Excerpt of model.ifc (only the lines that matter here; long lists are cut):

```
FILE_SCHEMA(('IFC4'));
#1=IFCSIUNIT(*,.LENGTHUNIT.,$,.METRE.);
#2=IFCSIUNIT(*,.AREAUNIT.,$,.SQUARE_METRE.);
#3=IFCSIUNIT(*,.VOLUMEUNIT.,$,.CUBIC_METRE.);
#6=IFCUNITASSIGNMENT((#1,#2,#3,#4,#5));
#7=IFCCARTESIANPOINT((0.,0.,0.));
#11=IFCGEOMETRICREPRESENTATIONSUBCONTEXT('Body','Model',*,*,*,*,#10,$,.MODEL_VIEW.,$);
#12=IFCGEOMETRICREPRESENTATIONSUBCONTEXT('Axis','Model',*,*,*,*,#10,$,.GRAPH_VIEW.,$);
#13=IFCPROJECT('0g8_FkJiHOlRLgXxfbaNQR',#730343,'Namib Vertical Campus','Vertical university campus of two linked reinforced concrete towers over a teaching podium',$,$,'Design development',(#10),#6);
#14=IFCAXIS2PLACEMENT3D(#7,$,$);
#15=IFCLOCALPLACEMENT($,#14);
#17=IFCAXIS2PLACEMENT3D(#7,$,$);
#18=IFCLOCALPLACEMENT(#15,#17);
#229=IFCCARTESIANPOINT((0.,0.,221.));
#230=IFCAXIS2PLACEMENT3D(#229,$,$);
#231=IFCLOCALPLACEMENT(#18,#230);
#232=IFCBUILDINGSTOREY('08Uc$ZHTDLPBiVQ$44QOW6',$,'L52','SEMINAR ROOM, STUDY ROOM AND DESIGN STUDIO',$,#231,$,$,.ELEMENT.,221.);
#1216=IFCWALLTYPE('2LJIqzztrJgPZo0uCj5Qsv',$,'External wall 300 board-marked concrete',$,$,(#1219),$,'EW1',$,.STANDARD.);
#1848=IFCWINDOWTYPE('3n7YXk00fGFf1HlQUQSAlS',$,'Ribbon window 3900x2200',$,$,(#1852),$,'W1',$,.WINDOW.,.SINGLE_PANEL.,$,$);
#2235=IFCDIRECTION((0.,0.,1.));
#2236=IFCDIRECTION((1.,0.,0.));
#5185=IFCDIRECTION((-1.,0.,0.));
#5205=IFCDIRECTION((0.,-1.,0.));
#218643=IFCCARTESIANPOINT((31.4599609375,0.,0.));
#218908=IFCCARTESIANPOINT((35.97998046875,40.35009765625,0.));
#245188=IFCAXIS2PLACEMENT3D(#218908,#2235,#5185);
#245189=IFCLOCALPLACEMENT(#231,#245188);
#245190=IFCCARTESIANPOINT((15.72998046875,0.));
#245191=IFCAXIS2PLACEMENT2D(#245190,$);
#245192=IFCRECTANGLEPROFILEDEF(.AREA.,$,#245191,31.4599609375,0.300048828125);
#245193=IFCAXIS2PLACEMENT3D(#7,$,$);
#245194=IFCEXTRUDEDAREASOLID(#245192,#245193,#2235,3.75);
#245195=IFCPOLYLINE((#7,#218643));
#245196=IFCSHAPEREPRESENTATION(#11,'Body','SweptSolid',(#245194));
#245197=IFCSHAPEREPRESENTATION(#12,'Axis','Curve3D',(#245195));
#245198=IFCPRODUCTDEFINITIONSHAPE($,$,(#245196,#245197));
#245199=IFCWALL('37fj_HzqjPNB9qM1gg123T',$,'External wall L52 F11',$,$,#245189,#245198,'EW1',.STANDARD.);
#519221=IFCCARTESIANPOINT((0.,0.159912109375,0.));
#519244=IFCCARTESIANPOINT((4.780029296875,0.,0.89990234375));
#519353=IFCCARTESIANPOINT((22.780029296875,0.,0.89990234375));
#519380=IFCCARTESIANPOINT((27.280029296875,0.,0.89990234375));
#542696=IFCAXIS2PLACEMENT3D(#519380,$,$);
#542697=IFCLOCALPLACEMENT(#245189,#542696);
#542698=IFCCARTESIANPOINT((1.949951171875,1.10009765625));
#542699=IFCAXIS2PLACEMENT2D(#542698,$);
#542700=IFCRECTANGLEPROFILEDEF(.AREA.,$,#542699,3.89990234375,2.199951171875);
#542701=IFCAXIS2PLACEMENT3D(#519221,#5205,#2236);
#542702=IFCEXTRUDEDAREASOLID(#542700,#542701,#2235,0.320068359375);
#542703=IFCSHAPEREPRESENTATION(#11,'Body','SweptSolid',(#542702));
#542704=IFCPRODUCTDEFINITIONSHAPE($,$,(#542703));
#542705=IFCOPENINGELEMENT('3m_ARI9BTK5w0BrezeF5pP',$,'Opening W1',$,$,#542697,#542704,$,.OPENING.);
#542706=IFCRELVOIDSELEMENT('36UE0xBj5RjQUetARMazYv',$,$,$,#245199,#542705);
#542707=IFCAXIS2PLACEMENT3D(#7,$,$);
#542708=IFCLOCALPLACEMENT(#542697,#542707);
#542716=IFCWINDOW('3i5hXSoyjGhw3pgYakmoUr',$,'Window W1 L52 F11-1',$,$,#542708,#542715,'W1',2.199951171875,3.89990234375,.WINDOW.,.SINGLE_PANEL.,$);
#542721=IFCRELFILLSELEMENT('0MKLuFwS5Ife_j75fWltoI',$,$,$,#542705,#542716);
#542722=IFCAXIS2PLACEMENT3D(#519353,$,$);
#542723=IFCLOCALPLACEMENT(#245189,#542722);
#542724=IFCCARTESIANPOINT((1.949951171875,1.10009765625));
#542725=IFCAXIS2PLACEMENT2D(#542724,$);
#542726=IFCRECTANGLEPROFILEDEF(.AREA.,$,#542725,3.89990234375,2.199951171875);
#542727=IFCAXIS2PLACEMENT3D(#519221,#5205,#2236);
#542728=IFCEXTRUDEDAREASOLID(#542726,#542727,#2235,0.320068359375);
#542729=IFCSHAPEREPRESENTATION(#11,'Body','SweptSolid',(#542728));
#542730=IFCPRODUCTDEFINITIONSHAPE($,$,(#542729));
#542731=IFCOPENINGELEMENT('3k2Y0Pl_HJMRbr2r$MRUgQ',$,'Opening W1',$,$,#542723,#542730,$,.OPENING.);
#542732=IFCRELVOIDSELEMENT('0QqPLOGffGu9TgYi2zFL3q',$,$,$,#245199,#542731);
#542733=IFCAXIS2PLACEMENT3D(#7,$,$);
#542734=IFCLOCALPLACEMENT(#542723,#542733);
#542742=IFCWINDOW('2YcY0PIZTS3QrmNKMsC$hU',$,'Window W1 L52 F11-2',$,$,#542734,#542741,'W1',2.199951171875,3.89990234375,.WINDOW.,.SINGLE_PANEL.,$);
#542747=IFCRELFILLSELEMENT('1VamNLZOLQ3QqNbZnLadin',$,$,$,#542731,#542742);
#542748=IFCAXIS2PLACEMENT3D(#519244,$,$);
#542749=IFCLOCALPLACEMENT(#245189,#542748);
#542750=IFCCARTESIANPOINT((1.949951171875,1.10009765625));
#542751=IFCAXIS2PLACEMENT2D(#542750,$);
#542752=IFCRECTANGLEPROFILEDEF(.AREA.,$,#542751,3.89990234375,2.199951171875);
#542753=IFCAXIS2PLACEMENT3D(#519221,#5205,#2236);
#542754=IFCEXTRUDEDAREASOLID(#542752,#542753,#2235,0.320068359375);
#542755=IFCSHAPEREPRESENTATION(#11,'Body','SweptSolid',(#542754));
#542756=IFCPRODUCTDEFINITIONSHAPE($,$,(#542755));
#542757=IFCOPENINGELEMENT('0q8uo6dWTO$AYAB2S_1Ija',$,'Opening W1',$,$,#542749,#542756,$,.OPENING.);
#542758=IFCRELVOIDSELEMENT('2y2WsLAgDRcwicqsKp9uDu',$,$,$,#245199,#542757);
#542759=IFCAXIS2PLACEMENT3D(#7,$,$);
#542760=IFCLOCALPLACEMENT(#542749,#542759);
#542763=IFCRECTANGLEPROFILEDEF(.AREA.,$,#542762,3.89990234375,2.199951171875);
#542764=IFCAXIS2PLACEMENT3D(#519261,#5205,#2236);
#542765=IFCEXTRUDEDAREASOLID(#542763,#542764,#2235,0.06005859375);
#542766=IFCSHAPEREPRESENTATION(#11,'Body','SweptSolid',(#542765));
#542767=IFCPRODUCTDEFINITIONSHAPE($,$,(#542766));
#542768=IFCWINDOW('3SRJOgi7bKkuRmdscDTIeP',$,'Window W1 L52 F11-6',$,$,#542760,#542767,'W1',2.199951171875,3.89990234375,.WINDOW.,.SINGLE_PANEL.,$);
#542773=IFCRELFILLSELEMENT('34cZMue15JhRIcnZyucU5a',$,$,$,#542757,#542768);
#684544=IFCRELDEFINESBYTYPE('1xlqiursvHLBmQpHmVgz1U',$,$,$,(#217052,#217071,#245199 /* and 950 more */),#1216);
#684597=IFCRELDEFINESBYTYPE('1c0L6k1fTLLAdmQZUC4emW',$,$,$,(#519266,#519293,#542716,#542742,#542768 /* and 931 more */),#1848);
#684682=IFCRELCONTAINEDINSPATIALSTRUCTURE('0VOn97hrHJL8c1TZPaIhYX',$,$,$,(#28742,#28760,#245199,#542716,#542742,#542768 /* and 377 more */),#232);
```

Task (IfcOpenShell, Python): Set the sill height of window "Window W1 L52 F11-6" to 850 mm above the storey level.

```python
import numpy as np
import ifcopenshell
import ifcopenshell.api.geometry
import ifcopenshell.geom
import ifcopenshell.util.element
import ifcopenshell.util.placement
import ifcopenshell.util.shape
import ifcopenshell.util.unit

model = ifcopenshell.open("model.ifc")
unit_scale = ifcopenshell.util.unit.calculate_unit_scale(model)

window = model.by_guid("3SRJOgi7bKkuRmdscDTIeP")
opening = window.FillsVoids[0].RelatingOpeningElement
storey = ifcopenshell.util.element.get_container(window, ifc_class="IfcBuildingStorey")
level = ifcopenshell.util.placement.get_local_placement(storey.ObjectPlacement)[2, 3]

# The opening's origin need not be at the sill, so measure its lowest point.
shape = ifcopenshell.geom.create_shape(ifcopenshell.geom.settings(), opening)
bottom = ifcopenshell.util.shape.get_shape_bottom_elevation(shape, shape.geometry) / unit_scale
dz = level + 0.85 - bottom

shift = np.array([0.0, 0.0, dz])
# The window is placed relative to its opening, so it follows when the opening moves.
matrix = ifcopenshell.util.placement.get_local_placement(opening.ObjectPlacement)
matrix[:3, 3] += shift
ifcopenshell.api.geometry.edit_object_placement(
    model, product=opening, matrix=matrix, is_si=False, should_transform_children=True
)

print(f"moved by {dz * unit_scale:+.3f} m")

model.write("model_rev.ifc")
```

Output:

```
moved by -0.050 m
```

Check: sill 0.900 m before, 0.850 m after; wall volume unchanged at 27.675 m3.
